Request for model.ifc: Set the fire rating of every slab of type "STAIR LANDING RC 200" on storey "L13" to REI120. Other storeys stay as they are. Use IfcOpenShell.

First a look at what the model holds.

```python
import ifcopenshell
import ifcopenshell.util.element

model = ifcopenshell.open("model.ifc")
print(model.schema)
storey = next(s for s in model.by_type("IfcBuildingStorey") if s.Name == "L13")
slabs = [e for e in ifcopenshell.util.element.get_decomposition(storey) if e.is_a("IfcSlab")]
seen = {}
for e in slabs:
    element_type = ifcopenshell.util.element.get_type(e)
    key = (element_type.Name if element_type != e and element_type else None, ifcopenshell.util.element.get_pset(e, "Pset_SlabCommon", "FireRating"))
    seen[key] = seen.get(key, 0) + 1
for (name, value), count in sorted(seen.items(), key=str):
    print(count, "x", name, "|", value)
```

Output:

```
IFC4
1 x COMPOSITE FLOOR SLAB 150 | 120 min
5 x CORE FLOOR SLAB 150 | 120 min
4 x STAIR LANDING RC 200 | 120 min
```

```python
import ifcopenshell
import ifcopenshell.api.pset
import ifcopenshell.util.element

model = ifcopenshell.open("model.ifc")

storey = next(s for s in model.by_type("IfcBuildingStorey") if s.Name == "L13")
slabs = [e for e in ifcopenshell.util.element.get_decomposition(storey) if e.is_a("IfcSlab")]

count = 0
for e in slabs:
    element_type = ifcopenshell.util.element.get_type(e)
    if element_type in (None, e) or element_type.Name != "STAIR LANDING RC 200":
        continue
    found = ifcopenshell.util.element.get_pset(e, "Pset_SlabCommon", should_inherit=False)
    if found:
        pset = model.by_id(found["id"])
        if len(ifcopenshell.util.element.get_elements_by_pset(pset)) > 1:
            pset = ifcopenshell.api.pset.unshare_pset(model, products=[e], pset=pset)[0]
    else:
        pset = ifcopenshell.api.pset.add_pset(model, product=e, name="Pset_SlabCommon")
    ifcopenshell.api.pset.edit_pset(model, pset=pset, properties={"FireRating": "REI120"})
    count += 1

print(count, "slabs updated")

model.write("model-out.ifc")
```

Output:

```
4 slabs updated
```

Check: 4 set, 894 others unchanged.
